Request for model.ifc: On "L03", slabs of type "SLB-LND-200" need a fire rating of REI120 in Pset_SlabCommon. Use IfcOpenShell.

First a look at what the model holds.

```python
import ifcopenshell
import ifcopenshell.util.element

model = ifcopenshell.open("model.ifc")
print(model.schema)
storey = next(s for s in model.by_type("IfcBuildingStorey") if s.Name == "L03")
slabs = [e for e in ifcopenshell.util.element.get_decomposition(storey) if e.is_a("IfcSlab")]
seen = {}
for e in slabs:
    element_type = ifcopenshell.util.element.get_type(e)
    key = (element_type.Name if element_type != e and element_type else None, ifcopenshell.util.element.get_pset(e, "Pset_SlabCommon", "FireRating"))
    seen[key] = seen.get(key, 0) + 1
for (name, value), count in sorted(seen.items(), key=str):
    print(count, "x", name, "|", value)
```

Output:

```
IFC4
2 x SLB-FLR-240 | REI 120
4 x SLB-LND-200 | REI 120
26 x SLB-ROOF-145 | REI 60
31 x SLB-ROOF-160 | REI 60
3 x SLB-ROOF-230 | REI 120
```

```python
import ifcopenshell
import ifcopenshell.api.pset
import ifcopenshell.util.element

model = ifcopenshell.open("model.ifc")

storey = next(s for s in model.by_type("IfcBuildingStorey") if s.Name == "L03")
slabs = [e for e in ifcopenshell.util.element.get_decomposition(storey) if e.is_a("IfcSlab")]

count = 0
for e in slabs:
    element_type = ifcopenshell.util.element.get_type(e)
    if element_type in (None, e) or element_type.Name != "SLB-LND-200":
        continue
    # add_pset returns the element's existing set when there is one.
    pset = ifcopenshell.api.pset.add_pset(model, product=e, name="Pset_SlabCommon")
    ifcopenshell.api.pset.edit_pset(model, pset=pset, properties={"FireRating": "REI120"})
    count += 1

print(count, "slabs updated")

model.write("model_v2.ifc")
```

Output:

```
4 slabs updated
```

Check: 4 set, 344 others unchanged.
